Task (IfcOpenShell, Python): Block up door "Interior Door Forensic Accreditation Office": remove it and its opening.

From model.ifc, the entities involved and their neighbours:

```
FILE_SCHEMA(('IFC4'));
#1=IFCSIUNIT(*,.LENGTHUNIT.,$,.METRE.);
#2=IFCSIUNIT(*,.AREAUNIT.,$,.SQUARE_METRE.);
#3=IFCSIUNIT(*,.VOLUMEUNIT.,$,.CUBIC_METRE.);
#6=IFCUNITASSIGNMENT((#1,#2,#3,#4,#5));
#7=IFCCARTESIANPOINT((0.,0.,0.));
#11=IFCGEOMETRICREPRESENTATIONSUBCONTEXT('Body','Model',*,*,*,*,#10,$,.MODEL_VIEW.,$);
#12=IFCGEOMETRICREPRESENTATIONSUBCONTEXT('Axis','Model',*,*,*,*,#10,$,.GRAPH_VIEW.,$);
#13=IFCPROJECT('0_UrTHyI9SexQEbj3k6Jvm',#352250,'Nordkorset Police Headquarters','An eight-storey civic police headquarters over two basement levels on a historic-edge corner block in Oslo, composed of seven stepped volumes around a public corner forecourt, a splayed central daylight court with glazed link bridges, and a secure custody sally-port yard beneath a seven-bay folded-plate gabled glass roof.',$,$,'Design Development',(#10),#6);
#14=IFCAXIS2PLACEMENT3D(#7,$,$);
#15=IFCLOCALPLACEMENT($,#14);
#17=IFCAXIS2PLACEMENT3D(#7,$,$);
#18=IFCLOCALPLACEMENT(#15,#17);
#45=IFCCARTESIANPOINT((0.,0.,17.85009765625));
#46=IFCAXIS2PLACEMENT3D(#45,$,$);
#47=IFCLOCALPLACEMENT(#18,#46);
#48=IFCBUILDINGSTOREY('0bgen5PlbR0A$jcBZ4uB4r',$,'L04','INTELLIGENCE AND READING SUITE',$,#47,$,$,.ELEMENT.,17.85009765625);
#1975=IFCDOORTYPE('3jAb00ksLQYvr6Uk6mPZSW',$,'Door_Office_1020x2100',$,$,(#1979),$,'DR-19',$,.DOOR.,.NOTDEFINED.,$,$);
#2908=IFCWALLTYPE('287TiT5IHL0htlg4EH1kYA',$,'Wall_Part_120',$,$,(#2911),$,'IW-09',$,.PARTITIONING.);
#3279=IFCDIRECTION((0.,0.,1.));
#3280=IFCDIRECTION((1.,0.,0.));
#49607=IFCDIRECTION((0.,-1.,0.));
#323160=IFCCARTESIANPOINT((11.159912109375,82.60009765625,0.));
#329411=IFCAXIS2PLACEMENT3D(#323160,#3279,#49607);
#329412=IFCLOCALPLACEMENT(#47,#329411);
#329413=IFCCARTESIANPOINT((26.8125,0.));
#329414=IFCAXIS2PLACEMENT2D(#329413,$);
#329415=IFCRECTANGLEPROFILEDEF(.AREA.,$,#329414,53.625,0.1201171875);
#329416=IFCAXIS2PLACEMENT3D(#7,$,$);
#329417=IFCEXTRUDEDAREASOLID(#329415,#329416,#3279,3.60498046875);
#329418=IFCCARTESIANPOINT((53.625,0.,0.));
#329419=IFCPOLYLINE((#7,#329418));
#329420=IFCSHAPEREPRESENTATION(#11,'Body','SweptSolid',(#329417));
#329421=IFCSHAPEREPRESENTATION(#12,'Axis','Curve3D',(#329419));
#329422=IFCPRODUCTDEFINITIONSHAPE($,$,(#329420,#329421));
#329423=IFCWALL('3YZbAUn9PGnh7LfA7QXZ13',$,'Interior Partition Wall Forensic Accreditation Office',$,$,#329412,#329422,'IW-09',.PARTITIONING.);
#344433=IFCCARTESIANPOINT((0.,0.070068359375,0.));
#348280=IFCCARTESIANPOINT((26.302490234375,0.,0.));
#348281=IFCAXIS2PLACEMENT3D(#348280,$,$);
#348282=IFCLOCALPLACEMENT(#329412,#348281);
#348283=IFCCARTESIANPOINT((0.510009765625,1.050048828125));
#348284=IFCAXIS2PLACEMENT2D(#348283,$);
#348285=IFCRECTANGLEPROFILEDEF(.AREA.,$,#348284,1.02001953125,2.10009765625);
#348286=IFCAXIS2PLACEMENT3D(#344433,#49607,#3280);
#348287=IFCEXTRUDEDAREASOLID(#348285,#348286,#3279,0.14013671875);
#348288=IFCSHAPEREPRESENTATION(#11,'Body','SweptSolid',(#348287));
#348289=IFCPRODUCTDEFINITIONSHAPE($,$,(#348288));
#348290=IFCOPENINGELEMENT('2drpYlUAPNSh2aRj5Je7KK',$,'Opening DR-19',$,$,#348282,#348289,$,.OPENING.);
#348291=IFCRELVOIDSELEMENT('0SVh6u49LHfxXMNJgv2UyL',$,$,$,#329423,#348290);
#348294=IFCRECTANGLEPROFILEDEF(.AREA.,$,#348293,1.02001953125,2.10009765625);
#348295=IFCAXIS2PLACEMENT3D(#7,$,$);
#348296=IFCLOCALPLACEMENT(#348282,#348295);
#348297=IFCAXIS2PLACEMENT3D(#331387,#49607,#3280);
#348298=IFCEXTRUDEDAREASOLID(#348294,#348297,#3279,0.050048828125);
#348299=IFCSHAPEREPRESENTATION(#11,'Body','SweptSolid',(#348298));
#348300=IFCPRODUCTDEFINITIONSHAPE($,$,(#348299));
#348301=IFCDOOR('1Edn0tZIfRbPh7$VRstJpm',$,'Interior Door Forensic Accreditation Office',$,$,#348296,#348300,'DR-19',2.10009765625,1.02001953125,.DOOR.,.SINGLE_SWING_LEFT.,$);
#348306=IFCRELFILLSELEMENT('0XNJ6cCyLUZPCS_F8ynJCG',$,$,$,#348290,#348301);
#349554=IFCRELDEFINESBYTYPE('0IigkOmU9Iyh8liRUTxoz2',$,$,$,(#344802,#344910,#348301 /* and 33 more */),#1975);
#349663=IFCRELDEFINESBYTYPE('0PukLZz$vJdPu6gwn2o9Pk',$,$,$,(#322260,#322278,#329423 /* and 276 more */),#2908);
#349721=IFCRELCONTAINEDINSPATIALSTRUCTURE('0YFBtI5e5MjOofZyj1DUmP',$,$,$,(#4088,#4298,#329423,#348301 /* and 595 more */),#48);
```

```python
import ifcopenshell
import ifcopenshell.api.feature
import ifcopenshell.api.root
import ifcopenshell.geom
import ifcopenshell.util.shape

model = ifcopenshell.open("model.ifc")
settings = ifcopenshell.geom.settings()


def volume(element):
    """Net volume in cubic metres, openings subtracted."""
    shape = ifcopenshell.geom.create_shape(settings, element)
    return ifcopenshell.util.shape.get_volume(shape.geometry)


door = model.by_guid("1Edn0tZIfRbPh7$VRstJpm")
opening = door.FillsVoids[0].RelatingOpeningElement
wall = opening.VoidsElements[0].RelatingBuildingElement
before = volume(wall)

ifcopenshell.api.root.remove_product(model, product=door)
ifcopenshell.api.feature.remove_feature(model, feature=opening)

after = volume(wall)

print(f"wall volume {before:.3f} -> {after:.3f} m3")

model.write("model-out.ifc")
```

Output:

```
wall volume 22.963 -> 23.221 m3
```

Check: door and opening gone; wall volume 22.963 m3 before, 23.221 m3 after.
